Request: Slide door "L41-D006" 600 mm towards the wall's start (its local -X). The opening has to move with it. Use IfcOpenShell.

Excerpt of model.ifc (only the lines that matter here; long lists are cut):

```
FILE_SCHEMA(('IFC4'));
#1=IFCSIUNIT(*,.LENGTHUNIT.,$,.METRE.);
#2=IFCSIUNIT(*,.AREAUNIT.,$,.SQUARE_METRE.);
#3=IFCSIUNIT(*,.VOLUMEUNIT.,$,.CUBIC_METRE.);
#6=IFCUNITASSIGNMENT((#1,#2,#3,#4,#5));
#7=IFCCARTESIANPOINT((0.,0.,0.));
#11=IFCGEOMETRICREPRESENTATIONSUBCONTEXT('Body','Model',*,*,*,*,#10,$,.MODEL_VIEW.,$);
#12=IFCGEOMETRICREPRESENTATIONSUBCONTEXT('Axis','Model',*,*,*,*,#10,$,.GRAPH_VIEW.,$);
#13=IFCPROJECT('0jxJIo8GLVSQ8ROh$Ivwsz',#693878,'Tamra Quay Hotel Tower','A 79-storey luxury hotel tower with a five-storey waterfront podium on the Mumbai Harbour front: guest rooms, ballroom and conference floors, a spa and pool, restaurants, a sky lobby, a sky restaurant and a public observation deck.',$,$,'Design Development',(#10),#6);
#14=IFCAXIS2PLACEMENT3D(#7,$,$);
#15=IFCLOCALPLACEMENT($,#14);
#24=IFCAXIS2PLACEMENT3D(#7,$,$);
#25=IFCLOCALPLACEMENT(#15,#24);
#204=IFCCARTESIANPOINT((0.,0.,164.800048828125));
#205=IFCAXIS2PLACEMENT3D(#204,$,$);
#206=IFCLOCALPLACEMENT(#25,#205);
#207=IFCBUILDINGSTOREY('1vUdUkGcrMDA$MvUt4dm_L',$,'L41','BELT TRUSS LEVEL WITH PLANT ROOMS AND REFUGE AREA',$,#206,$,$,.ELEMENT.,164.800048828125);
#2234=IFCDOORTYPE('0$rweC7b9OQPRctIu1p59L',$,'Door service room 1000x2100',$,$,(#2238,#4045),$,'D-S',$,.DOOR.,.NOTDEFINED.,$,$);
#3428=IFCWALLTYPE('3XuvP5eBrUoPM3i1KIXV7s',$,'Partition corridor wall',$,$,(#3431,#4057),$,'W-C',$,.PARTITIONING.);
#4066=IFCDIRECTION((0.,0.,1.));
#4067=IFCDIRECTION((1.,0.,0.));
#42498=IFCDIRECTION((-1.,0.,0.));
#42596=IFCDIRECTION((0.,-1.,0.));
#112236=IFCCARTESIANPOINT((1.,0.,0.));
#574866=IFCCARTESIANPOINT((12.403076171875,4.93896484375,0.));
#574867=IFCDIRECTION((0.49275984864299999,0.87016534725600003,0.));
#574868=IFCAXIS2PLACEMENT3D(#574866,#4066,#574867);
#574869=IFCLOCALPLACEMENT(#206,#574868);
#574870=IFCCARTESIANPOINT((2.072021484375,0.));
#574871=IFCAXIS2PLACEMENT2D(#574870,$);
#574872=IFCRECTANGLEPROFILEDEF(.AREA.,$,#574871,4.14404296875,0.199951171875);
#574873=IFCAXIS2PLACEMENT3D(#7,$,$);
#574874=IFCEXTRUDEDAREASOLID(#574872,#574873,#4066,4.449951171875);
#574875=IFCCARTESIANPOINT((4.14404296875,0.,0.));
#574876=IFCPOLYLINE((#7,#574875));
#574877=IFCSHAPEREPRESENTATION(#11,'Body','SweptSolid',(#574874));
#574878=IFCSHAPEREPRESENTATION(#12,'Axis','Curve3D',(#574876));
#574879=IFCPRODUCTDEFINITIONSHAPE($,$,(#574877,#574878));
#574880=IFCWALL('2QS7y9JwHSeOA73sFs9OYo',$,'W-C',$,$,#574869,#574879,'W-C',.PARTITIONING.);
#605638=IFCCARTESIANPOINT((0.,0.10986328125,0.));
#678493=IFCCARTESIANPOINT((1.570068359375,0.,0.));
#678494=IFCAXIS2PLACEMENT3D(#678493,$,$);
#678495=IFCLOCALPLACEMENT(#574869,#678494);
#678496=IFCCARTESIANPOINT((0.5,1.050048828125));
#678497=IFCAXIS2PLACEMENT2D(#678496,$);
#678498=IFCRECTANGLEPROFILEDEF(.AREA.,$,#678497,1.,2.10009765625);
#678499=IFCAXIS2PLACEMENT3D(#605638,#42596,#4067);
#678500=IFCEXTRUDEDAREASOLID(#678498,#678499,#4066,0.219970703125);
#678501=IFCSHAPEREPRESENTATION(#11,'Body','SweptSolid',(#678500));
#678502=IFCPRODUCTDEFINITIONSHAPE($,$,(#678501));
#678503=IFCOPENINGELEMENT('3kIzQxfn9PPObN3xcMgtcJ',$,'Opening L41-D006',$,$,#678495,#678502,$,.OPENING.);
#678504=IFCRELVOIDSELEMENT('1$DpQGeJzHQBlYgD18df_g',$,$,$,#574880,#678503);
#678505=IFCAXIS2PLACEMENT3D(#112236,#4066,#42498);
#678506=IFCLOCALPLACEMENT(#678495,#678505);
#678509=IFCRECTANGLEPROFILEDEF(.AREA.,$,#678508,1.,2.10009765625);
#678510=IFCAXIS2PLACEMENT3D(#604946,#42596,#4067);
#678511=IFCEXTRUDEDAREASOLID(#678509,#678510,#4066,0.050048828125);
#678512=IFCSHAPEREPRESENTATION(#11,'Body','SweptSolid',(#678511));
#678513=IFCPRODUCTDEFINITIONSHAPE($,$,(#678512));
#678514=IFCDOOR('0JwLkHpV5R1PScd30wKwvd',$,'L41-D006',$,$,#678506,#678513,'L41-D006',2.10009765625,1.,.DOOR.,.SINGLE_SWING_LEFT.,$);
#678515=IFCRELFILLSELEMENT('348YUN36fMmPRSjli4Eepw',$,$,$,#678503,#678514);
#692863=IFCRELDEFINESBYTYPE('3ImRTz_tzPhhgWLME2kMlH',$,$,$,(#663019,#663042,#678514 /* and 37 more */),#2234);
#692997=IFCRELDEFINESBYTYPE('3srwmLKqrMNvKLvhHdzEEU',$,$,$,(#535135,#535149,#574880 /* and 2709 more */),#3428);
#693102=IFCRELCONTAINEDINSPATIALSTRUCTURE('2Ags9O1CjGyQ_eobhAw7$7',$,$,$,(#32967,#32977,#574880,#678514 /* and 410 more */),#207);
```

```python
import ifcopenshell
import ifcopenshell.api.geometry
import ifcopenshell.util.placement

model = ifcopenshell.open("model.ifc")

door = model.by_id(678514)
opening = door.FillsVoids[0].RelatingOpeningElement
wall = opening.VoidsElements[0].RelatingBuildingElement

wall_matrix = ifcopenshell.util.placement.get_local_placement(wall.ObjectPlacement)
shift = wall_matrix[:3, 0] * -0.6
before = ifcopenshell.util.placement.get_local_placement(door.ObjectPlacement)[:3, 3].copy()

# The door is placed relative to its opening, so it follows when the opening moves.
matrix = ifcopenshell.util.placement.get_local_placement(opening.ObjectPlacement)
matrix[:3, 3] += shift
ifcopenshell.api.geometry.edit_object_placement(
    model, product=opening, matrix=matrix, is_si=False, should_transform_children=True
)

after = ifcopenshell.util.placement.get_local_placement(door.ObjectPlacement)[:3, 3]
print("door moved by", (after - before).round(3) + 0.0)

model.write("model-out.ifc")
```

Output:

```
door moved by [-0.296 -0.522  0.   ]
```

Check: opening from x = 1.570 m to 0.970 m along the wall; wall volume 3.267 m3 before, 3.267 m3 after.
